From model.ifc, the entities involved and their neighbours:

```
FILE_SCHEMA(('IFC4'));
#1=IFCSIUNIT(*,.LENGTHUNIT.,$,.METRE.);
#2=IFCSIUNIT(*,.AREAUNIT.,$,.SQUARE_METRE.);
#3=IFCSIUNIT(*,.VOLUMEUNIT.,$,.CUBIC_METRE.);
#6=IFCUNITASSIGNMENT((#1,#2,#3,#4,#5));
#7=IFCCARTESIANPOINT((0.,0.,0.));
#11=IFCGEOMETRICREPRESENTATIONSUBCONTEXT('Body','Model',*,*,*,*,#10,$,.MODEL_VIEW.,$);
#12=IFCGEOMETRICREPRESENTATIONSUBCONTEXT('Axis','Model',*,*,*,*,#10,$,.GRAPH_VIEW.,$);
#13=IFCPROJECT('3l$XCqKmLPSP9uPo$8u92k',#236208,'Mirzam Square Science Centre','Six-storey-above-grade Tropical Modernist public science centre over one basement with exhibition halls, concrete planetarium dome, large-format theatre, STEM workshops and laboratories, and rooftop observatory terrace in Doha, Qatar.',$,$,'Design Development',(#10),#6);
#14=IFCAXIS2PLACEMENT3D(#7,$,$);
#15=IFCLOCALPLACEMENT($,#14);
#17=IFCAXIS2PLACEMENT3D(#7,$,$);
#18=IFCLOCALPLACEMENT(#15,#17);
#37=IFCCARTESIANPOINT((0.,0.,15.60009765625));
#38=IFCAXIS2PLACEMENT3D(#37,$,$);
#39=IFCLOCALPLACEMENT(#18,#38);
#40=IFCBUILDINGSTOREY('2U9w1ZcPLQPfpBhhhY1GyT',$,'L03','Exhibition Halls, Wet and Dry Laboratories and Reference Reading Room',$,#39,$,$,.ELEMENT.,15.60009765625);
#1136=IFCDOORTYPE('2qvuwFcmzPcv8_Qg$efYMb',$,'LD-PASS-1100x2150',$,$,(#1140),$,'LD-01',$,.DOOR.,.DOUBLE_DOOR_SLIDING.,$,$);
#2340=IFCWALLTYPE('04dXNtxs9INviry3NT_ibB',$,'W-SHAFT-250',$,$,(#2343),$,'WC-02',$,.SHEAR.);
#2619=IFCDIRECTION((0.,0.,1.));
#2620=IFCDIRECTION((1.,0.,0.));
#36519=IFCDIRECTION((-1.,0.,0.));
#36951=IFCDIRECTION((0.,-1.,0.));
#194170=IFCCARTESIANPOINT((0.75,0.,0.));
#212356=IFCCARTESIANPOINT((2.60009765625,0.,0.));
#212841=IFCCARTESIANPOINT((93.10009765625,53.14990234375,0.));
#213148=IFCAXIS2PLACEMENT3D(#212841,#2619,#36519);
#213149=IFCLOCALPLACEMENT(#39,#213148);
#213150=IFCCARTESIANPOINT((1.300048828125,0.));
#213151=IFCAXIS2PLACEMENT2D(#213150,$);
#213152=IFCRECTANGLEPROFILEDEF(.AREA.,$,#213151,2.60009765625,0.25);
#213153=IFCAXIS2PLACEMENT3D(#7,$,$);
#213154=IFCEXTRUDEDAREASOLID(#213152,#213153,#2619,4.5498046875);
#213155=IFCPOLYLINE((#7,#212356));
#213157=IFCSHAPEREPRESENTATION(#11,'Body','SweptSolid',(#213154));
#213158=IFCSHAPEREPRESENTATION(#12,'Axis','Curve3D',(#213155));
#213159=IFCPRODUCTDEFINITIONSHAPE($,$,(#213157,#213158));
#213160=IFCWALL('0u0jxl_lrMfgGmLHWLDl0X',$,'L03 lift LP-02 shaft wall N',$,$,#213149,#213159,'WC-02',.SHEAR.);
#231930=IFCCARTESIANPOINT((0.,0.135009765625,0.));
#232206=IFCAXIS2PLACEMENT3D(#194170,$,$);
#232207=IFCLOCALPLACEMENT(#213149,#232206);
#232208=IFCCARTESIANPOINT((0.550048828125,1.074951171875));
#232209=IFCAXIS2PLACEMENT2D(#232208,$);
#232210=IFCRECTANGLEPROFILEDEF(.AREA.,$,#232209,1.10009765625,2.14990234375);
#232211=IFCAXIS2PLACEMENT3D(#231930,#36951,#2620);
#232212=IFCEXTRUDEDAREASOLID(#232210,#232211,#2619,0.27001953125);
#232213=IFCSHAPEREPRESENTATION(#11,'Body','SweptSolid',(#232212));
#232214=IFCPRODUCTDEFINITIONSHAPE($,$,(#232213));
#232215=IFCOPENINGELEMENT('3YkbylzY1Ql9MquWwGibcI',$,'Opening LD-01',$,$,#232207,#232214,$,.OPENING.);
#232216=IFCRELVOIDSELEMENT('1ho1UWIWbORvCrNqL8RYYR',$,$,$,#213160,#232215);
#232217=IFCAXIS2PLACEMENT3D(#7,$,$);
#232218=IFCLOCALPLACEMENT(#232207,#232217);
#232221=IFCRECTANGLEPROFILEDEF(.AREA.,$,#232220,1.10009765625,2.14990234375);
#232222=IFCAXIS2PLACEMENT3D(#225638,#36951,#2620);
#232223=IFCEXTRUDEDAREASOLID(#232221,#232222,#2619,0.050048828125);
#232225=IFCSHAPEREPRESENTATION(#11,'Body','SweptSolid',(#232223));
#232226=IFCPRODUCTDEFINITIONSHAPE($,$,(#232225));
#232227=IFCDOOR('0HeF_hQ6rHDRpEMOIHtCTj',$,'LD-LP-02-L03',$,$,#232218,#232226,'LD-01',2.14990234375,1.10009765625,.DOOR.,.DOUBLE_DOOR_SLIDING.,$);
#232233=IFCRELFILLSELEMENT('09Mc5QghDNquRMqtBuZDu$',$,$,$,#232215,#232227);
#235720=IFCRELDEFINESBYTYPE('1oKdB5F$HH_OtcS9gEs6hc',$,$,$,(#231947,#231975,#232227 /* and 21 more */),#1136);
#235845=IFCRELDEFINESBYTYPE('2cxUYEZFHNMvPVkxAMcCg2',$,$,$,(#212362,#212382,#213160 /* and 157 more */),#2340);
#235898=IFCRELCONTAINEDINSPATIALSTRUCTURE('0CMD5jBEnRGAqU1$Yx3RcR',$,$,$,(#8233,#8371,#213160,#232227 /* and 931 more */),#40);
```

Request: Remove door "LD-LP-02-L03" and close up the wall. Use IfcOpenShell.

```python
import ifcopenshell
import ifcopenshell.api.feature
import ifcopenshell.api.root
import ifcopenshell.geom
import ifcopenshell.util.shape

model = ifcopenshell.open("model.ifc")
settings = ifcopenshell.geom.settings()


def volume(element):
    """Net volume in cubic metres, openings subtracted."""
    shape = ifcopenshell.geom.create_shape(settings, element)
    return ifcopenshell.util.shape.get_volume(shape.geometry)


door = model.by_id(232227)
opening = door.FillsVoids[0].RelatingOpeningElement
wall = opening.VoidsElements[0].RelatingBuildingElement
before = volume(wall)

ifcopenshell.api.root.remove_product(model, product=door)
ifcopenshell.api.feature.remove_feature(model, feature=opening)

after = volume(wall)

print(f"wall volume {before:.3f} -> {after:.3f} m3")

model.write("model-out.ifc")
```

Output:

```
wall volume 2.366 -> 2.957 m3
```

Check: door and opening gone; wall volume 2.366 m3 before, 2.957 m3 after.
